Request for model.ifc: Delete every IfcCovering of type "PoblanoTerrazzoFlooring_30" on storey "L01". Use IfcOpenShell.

First a look at what the model holds.

```python
import ifcopenshell
import ifcopenshell.util.element

model = ifcopenshell.open("model.ifc")
print(model.schema)
storey = next(s for s in model.by_type("IfcBuildingStorey") if s.Name == "L01")
coverings = [e for e in ifcopenshell.util.element.get_decomposition(storey) if e.is_a("IfcCovering")]
seen = {}
for e in coverings:
    element_type = ifcopenshell.util.element.get_type(e)
    name = element_type.Name if element_type not in (None, e) else None
    seen[name] = seen.get(name, 0) + 1
for name, count in sorted(seen.items(), key=str):
    print(count, "x", name)
```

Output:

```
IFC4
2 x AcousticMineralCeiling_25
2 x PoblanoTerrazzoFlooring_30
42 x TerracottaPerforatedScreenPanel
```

```python
import ifcopenshell
import ifcopenshell.api.root
import ifcopenshell.util.element

model = ifcopenshell.open("model.ifc")

storey = next(s for s in model.by_type("IfcBuildingStorey") if s.Name == "L01")
coverings = [e for e in ifcopenshell.util.element.get_decomposition(storey) if e.is_a("IfcCovering")]
targets = [e for e in coverings if (t := ifcopenshell.util.element.get_type(e)) not in (None, e) and t.Name == "PoblanoTerrazzoFlooring_30"]

for e in targets:
    ifcopenshell.api.root.remove_product(model, product=e)
print(len(targets), "removed")

model.write("model-out.ifc")
```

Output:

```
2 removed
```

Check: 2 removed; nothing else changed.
